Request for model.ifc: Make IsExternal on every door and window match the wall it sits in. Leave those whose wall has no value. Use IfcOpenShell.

First a look at what the model holds.

```python
import ifcopenshell
import ifcopenshell.util.element

model = ifcopenshell.open("model.ifc")
print(model.schema)
seen = {}
for e in model.by_type("IfcDoor") + model.by_type("IfcWindow"):
    if not e.FillsVoids:
        continue
    host = e.FillsVoids[0].RelatingOpeningElement.VoidsElements[0].RelatingBuildingElement
    own = ifcopenshell.util.element.get_pset(e, f"Pset_{e.is_a()[3:].removesuffix('StandardCase')}Common", "IsExternal")
    wall = ifcopenshell.util.element.get_pset(host, "Pset_WallCommon", "IsExternal")
    seen[e.is_a(), own, wall] = seen.get((e.is_a(), own, wall), 0) + 1
for (cls, own, wall), count in sorted(seen.items(), key=str):
    print(count, cls, "IsExternal:", own, "| host wall:", wall)
```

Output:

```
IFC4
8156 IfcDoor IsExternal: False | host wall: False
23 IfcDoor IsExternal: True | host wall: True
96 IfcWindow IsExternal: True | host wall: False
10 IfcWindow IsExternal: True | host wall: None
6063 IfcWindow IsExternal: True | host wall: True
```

```python
import ifcopenshell
import ifcopenshell.api.pset
import ifcopenshell.util.element

model = ifcopenshell.open("model.ifc")

count = 0
for ifc_class, pset_name in (("IfcDoor", "Pset_DoorCommon"), ("IfcWindow", "Pset_WindowCommon")):
    for e in model.by_type(ifc_class):
        if not e.FillsVoids:
            continue
        host = e.FillsVoids[0].RelatingOpeningElement.VoidsElements[0].RelatingBuildingElement
        external = ifcopenshell.util.element.get_pset(host, "Pset_WallCommon", "IsExternal")
        if external is None or ifcopenshell.util.element.get_pset(e, pset_name, "IsExternal") == external:
            continue
        found = ifcopenshell.util.element.get_pset(e, pset_name, should_inherit=False)
        if found:
            pset = model.by_id(found["id"])
            if len(ifcopenshell.util.element.get_elements_by_pset(pset)) > 1:
                pset = ifcopenshell.api.pset.unshare_pset(model, products=[e], pset=pset)[0]
        else:
            pset = ifcopenshell.api.pset.add_pset(model, product=e, name=pset_name)
        ifcopenshell.api.pset.edit_pset(model, pset=pset, properties={"IsExternal": external})
        count += 1

print(count, "updated")

model.write("model_updated.ifc")
```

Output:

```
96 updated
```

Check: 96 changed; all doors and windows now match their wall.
